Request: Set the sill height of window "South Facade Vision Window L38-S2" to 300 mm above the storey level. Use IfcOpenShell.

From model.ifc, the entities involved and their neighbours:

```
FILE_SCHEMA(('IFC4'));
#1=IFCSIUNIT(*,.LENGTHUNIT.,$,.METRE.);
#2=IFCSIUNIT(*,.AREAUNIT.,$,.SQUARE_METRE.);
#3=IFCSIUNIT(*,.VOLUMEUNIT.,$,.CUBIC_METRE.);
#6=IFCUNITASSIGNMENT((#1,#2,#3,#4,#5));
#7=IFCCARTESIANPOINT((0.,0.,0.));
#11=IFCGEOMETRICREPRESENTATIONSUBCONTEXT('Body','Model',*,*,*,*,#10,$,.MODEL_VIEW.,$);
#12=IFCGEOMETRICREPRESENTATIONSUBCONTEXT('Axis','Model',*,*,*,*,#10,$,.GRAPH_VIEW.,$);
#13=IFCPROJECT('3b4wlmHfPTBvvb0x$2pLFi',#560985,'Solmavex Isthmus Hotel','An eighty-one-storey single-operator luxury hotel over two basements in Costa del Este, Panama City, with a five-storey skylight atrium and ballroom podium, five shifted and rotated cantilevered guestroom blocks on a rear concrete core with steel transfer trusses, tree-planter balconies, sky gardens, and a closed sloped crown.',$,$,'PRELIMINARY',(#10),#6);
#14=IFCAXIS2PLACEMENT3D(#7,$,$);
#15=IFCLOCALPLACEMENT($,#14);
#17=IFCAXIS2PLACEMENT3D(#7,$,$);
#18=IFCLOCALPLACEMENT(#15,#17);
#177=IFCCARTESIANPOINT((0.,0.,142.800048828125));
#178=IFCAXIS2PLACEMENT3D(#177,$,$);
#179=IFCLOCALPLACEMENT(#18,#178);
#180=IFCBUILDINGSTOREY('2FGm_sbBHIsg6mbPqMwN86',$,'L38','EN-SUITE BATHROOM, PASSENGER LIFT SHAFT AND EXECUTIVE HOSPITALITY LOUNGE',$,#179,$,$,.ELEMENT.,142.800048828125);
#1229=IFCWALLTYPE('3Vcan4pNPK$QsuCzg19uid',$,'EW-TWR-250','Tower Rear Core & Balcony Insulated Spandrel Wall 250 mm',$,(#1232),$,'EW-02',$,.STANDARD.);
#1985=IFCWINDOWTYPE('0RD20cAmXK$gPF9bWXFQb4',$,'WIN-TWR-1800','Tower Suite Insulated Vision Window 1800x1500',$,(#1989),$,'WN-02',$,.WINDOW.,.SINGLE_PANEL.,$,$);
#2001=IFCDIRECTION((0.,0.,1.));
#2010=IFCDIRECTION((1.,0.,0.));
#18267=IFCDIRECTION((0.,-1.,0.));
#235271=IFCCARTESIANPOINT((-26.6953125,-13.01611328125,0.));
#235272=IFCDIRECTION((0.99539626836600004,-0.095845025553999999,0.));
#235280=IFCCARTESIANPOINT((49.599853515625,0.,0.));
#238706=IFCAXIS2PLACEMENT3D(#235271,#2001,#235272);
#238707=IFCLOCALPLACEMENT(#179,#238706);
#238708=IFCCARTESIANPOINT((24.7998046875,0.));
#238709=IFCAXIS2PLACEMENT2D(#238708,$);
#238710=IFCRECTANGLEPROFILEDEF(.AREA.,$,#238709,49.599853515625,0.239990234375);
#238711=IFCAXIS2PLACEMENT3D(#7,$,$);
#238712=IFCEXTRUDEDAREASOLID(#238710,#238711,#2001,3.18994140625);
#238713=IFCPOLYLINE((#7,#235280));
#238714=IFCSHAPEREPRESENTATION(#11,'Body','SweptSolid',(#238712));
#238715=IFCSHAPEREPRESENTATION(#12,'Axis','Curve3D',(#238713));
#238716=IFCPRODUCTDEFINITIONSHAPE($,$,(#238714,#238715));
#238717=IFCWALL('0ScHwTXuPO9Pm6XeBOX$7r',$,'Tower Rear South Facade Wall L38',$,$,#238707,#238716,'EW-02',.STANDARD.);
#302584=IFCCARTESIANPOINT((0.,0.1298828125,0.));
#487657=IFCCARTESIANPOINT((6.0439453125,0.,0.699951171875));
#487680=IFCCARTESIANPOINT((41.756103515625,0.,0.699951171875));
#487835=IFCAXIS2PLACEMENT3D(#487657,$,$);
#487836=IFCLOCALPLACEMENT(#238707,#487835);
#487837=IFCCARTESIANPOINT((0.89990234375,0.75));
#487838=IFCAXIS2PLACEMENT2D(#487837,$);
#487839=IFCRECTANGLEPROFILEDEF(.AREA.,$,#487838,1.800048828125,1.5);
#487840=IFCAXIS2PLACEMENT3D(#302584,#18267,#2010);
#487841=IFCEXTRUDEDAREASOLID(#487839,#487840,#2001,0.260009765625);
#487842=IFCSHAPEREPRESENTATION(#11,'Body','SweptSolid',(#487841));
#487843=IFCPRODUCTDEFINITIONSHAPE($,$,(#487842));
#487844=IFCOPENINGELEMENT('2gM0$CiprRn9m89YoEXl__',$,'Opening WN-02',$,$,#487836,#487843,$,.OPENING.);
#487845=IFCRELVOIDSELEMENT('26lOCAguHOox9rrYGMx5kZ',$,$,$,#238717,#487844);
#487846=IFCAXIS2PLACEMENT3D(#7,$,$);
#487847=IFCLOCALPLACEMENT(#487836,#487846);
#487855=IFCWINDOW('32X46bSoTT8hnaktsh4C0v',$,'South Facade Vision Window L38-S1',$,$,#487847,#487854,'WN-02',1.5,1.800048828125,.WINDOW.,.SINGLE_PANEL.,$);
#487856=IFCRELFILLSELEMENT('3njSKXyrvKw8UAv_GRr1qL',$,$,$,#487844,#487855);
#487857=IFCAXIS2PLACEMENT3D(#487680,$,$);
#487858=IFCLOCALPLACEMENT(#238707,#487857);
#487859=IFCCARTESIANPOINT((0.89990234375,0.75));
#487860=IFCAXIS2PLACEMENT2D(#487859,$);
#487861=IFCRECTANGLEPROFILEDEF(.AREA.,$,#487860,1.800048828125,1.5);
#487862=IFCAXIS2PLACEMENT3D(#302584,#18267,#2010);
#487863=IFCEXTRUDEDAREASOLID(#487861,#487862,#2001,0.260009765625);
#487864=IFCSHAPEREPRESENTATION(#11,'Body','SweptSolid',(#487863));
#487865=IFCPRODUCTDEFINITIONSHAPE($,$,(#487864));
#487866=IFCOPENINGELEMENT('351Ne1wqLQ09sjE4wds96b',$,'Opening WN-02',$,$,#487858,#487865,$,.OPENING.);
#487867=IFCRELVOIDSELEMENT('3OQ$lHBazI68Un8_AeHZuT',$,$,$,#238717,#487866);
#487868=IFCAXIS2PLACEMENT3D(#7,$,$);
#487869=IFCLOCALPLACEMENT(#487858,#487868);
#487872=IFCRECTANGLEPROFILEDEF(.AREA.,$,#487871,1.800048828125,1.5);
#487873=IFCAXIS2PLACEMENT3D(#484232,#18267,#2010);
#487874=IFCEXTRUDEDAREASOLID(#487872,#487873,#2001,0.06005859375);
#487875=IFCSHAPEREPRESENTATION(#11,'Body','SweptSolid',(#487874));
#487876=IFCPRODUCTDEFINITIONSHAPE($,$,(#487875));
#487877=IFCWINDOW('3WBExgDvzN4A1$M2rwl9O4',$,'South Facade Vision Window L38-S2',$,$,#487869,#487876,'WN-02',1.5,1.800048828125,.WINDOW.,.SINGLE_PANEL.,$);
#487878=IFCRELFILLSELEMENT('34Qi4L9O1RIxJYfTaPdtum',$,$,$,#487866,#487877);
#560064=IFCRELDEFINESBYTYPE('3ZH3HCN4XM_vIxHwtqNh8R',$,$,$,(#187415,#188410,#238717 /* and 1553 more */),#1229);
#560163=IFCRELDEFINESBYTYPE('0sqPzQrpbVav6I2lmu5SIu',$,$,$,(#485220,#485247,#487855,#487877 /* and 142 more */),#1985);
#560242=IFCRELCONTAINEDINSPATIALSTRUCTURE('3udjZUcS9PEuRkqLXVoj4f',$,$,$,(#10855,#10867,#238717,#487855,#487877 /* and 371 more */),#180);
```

```python
import numpy as np
import ifcopenshell
import ifcopenshell.api.geometry
import ifcopenshell.geom
import ifcopenshell.util.element
import ifcopenshell.util.placement
import ifcopenshell.util.shape
import ifcopenshell.util.unit

model = ifcopenshell.open("model.ifc")
unit_scale = ifcopenshell.util.unit.calculate_unit_scale(model)

window = model.by_id(487877)
opening = window.FillsVoids[0].RelatingOpeningElement
storey = ifcopenshell.util.element.get_container(window, ifc_class="IfcBuildingStorey")
level = ifcopenshell.util.placement.get_local_placement(storey.ObjectPlacement)[2, 3]

# The opening's origin need not be at the sill, so measure its lowest point.
shape = ifcopenshell.geom.create_shape(ifcopenshell.geom.settings(), opening)
bottom = ifcopenshell.util.shape.get_shape_bottom_elevation(shape, shape.geometry) / unit_scale
dz = level + 0.3 / unit_scale - bottom

shift = np.array([0.0, 0.0, dz])
# The window is placed relative to its opening, so it follows when the opening moves.
matrix = ifcopenshell.util.placement.get_local_placement(opening.ObjectPlacement)
matrix[:3, 3] += shift
ifcopenshell.api.geometry.edit_object_placement(
    model, product=opening, matrix=matrix, is_si=False, should_transform_children=True
)

print(f"moved by {dz * unit_scale:+.3f} m")

model.write("model_rev.ifc")
```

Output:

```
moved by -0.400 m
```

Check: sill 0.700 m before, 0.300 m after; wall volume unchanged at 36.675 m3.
